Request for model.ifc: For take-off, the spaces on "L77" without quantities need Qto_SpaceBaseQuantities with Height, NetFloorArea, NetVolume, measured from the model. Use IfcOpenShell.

First a look at what the model holds.

```python
import ifcopenshell
import ifcopenshell.util.element
import ifcopenshell.util.unit

model = ifcopenshell.open("model.ifc")
print(model.schema)
for unit_type in ("LENGTHUNIT", "AREAUNIT", "VOLUMEUNIT"):
    print(unit_type, ifcopenshell.util.unit.calculate_unit_scale(model, unit_type))
storey = next(s for s in model.by_type("IfcBuildingStorey") if s.Name == "L77")
spaces = [e for e in ifcopenshell.util.element.get_decomposition(storey) if e.is_a("IfcSpace")]
for e in sorted(spaces, key=lambda e: e.id()):
    print(e.id(), e.is_a(), e.Name, list(ifcopenshell.util.element.get_psets(e, qtos_only=True)), sep=" | ")
```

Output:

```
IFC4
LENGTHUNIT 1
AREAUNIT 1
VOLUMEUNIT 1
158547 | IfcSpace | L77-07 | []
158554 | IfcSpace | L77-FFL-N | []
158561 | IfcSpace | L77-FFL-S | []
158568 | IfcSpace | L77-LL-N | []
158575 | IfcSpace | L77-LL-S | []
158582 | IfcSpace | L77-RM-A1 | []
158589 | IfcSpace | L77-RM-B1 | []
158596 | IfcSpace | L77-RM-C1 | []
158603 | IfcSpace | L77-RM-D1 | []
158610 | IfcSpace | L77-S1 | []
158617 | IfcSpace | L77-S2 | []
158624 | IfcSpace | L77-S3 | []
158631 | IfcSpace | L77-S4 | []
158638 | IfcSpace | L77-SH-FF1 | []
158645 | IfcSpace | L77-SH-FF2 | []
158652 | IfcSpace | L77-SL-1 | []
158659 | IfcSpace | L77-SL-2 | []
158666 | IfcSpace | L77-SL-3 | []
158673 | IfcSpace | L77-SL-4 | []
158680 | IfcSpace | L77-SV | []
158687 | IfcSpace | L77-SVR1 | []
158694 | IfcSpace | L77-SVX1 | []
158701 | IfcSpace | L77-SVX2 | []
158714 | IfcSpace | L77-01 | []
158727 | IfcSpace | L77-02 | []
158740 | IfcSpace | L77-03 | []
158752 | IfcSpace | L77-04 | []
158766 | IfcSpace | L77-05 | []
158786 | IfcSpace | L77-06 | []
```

```python
import ifcopenshell
import ifcopenshell.api.pset
import ifcopenshell.geom
import ifcopenshell.util.element
import ifcopenshell.util.shape
import ifcopenshell.util.unit

model = ifcopenshell.open("model.ifc")
unit_scale = ifcopenshell.util.unit.calculate_unit_scale(model)
area_scale = ifcopenshell.util.unit.calculate_unit_scale(model, "AREAUNIT")
volume_scale = ifcopenshell.util.unit.calculate_unit_scale(model, "VOLUMEUNIT")
settings = ifcopenshell.geom.settings()

storey = next(s for s in model.by_type("IfcBuildingStorey") if s.Name == "L77")
spaces = [e for e in ifcopenshell.util.element.get_decomposition(storey) if e.is_a("IfcSpace")]

for e in sorted(spaces, key=lambda e: e.id()):
    if ifcopenshell.util.element.get_psets(e, qtos_only=True, should_inherit=False):
        continue
    # Geometry comes back in metres, in the element's own axes.
    shape = ifcopenshell.geom.create_shape(settings, e)
    values = {
        "Height": ifcopenshell.util.shape.get_z(shape.geometry) / unit_scale,
        "NetFloorArea": ifcopenshell.util.shape.get_footprint_area(shape.geometry) / area_scale,
        "NetVolume": ifcopenshell.util.shape.get_volume(shape.geometry) / volume_scale,
    }
    qto = ifcopenshell.api.pset.add_qto(model, product=e, name="Qto_SpaceBaseQuantities")
    ifcopenshell.api.pset.edit_qto(model, qto=qto, properties=values)
    print(e.id(), {k: round(v, 3) for k, v in values.items()})

model.write("model_updated.ifc")
```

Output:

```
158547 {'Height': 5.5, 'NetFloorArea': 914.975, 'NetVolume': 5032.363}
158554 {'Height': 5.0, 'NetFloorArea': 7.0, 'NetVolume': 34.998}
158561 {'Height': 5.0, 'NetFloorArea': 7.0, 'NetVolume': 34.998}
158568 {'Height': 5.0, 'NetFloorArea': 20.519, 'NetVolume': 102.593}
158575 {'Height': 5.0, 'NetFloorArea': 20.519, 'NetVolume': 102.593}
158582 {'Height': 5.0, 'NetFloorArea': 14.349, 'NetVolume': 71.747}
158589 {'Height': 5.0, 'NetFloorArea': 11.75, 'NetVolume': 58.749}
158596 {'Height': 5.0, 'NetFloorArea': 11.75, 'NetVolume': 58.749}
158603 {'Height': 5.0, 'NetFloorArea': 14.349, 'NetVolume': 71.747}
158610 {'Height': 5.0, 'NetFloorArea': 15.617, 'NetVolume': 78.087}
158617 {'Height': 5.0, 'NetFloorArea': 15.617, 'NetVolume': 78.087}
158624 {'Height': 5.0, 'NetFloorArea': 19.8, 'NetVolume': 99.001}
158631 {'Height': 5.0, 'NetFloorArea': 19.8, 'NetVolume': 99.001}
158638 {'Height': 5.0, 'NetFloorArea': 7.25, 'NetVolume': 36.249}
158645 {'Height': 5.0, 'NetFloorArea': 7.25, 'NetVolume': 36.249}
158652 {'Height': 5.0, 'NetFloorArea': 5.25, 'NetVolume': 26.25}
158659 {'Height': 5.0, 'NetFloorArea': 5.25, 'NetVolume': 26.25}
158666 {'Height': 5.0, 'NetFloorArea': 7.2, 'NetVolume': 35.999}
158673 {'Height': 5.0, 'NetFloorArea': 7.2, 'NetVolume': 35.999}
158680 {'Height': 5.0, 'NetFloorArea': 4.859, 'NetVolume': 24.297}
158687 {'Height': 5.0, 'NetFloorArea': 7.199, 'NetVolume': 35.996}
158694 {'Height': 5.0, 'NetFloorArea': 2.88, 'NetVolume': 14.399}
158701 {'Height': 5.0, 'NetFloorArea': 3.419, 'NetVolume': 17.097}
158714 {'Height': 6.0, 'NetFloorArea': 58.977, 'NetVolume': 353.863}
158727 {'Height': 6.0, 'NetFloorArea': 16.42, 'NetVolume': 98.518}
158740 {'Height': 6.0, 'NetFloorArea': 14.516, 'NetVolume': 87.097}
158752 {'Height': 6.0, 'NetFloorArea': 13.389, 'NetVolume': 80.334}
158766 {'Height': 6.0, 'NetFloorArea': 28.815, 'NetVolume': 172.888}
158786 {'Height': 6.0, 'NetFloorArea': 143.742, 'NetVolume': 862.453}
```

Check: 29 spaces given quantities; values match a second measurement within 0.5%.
